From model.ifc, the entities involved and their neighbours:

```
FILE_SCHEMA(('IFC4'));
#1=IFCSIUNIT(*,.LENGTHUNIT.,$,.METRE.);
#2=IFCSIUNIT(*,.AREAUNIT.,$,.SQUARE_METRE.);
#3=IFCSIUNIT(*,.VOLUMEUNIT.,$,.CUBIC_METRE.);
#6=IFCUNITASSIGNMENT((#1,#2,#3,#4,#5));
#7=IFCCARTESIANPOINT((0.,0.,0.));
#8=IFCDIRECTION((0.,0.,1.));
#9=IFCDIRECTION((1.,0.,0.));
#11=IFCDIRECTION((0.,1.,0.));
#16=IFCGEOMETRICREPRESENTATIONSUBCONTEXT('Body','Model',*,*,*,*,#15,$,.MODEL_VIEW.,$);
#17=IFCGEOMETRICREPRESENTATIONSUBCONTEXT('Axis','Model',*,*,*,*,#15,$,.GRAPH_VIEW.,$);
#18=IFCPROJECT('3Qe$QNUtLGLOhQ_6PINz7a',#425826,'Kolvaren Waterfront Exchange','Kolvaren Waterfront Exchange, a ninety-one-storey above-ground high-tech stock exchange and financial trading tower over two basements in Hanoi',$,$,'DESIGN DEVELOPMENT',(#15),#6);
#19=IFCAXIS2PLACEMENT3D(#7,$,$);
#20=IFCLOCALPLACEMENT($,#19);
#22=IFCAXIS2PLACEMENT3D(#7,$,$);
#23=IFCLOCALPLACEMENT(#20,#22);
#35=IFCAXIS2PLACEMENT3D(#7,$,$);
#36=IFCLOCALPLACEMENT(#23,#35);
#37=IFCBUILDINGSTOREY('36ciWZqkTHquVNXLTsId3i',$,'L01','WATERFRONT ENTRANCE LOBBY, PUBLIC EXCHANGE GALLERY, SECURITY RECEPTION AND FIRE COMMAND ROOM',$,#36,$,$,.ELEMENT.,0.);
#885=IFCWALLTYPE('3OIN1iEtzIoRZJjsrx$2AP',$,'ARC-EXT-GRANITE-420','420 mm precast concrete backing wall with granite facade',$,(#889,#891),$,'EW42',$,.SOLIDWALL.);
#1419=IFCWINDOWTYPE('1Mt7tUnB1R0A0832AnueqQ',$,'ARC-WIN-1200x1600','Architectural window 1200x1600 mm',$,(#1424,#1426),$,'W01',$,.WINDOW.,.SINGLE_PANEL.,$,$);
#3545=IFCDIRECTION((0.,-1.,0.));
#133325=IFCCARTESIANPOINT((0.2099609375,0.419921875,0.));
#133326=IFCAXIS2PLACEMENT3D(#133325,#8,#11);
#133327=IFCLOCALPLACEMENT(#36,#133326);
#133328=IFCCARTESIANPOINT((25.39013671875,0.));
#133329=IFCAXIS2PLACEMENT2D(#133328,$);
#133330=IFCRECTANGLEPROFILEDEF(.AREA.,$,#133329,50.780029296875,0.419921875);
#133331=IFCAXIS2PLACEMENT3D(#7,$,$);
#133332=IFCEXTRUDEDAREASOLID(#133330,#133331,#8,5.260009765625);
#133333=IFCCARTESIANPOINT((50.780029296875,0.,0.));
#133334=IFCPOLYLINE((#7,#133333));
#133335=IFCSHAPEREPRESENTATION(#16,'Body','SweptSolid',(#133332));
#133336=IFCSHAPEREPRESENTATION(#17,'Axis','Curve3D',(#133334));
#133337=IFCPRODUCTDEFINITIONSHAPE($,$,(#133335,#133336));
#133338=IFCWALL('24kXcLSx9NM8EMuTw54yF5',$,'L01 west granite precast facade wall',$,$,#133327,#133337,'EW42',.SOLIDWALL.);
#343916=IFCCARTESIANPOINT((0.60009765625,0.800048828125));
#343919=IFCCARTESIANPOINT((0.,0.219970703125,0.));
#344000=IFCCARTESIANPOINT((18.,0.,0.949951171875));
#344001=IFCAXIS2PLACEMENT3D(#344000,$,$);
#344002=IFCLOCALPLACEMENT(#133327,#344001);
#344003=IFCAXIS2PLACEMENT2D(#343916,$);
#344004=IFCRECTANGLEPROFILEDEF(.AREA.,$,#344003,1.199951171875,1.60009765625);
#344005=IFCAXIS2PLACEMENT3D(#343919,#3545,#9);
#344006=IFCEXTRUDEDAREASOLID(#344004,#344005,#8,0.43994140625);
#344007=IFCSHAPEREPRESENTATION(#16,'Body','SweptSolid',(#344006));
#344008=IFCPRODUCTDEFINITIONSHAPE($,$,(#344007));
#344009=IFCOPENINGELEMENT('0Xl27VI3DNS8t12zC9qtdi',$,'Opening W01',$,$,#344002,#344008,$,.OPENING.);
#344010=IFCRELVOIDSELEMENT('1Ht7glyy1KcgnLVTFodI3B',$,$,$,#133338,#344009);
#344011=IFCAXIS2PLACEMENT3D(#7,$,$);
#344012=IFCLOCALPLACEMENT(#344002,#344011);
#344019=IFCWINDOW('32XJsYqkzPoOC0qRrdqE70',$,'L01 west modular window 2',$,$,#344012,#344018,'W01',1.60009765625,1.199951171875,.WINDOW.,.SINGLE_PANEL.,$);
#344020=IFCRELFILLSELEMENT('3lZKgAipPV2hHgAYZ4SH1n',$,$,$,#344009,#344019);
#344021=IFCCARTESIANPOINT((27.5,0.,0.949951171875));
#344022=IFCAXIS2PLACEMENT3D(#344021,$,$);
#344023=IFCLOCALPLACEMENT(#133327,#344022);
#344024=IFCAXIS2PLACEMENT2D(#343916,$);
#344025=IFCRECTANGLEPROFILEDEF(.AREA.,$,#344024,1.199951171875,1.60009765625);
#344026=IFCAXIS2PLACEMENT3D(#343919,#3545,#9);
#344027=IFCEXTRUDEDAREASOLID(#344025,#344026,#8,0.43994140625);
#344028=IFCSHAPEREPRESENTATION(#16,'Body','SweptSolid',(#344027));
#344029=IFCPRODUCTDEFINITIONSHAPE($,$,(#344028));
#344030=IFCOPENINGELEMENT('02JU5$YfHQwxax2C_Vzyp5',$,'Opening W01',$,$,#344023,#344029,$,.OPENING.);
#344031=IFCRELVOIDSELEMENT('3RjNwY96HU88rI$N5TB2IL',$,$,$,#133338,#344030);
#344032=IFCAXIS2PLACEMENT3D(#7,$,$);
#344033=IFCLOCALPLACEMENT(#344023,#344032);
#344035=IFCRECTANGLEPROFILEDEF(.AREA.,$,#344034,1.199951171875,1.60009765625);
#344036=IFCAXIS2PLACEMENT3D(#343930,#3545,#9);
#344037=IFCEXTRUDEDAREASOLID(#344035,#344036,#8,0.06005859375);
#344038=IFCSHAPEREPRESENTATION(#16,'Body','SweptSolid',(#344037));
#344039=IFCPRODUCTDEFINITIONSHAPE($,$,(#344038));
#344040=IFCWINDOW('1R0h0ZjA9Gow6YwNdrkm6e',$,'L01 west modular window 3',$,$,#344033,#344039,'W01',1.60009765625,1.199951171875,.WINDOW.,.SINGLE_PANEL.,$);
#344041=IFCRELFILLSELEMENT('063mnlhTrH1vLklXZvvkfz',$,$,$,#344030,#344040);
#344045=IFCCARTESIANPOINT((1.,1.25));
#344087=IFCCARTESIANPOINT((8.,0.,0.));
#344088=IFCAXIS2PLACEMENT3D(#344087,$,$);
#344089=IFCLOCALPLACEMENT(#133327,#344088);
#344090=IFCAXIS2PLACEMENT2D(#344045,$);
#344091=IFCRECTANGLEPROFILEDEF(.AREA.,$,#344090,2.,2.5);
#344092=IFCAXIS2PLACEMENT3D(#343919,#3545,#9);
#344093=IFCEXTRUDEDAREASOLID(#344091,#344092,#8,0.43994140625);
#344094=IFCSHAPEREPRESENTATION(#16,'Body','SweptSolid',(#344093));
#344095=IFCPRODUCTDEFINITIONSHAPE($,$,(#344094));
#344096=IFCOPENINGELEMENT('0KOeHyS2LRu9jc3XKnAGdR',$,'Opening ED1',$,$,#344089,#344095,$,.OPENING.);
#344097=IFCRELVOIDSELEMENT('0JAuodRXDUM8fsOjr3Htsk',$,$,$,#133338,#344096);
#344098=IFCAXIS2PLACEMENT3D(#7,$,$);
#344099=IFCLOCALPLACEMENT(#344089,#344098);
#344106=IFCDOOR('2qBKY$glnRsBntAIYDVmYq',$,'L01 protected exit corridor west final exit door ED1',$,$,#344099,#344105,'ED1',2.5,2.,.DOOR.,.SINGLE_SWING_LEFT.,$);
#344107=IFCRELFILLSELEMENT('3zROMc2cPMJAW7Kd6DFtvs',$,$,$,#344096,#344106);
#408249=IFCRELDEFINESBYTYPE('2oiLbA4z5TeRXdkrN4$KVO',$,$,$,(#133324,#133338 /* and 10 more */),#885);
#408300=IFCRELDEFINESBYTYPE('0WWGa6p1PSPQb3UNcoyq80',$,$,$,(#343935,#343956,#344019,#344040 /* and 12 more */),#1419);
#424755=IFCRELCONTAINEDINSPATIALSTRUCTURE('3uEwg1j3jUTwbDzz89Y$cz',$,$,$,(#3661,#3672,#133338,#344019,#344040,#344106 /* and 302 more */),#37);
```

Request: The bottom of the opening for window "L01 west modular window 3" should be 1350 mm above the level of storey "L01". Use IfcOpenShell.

```python
import numpy as np
import ifcopenshell
import ifcopenshell.api.geometry
import ifcopenshell.geom
import ifcopenshell.util.element
import ifcopenshell.util.placement
import ifcopenshell.util.shape
import ifcopenshell.util.unit

model = ifcopenshell.open("model.ifc")
unit_scale = ifcopenshell.util.unit.calculate_unit_scale(model)

window = model.by_id(344040)
opening = window.FillsVoids[0].RelatingOpeningElement
storey = ifcopenshell.util.element.get_container(window, ifc_class="IfcBuildingStorey")
level = ifcopenshell.util.placement.get_local_placement(storey.ObjectPlacement)[2, 3]

# The opening's origin need not be at the sill, so measure its lowest point.
shape = ifcopenshell.geom.create_shape(ifcopenshell.geom.settings(), opening)
bottom = ifcopenshell.util.shape.get_shape_bottom_elevation(shape, shape.geometry) / unit_scale
dz = level + 1.35 / unit_scale - bottom

shift = np.array([0.0, 0.0, dz])
# The window is placed relative to its opening, so it follows when the opening moves.
matrix = ifcopenshell.util.placement.get_local_placement(opening.ObjectPlacement)
matrix[:3, 3] += shift
ifcopenshell.api.geometry.edit_object_placement(
    model, product=opening, matrix=matrix, is_si=False, should_transform_children=True
)

print(f"moved by {dz * unit_scale:+.3f} m")

model.write("model_updated.ifc")
```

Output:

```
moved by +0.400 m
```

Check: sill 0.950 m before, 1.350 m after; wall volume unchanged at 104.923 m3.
